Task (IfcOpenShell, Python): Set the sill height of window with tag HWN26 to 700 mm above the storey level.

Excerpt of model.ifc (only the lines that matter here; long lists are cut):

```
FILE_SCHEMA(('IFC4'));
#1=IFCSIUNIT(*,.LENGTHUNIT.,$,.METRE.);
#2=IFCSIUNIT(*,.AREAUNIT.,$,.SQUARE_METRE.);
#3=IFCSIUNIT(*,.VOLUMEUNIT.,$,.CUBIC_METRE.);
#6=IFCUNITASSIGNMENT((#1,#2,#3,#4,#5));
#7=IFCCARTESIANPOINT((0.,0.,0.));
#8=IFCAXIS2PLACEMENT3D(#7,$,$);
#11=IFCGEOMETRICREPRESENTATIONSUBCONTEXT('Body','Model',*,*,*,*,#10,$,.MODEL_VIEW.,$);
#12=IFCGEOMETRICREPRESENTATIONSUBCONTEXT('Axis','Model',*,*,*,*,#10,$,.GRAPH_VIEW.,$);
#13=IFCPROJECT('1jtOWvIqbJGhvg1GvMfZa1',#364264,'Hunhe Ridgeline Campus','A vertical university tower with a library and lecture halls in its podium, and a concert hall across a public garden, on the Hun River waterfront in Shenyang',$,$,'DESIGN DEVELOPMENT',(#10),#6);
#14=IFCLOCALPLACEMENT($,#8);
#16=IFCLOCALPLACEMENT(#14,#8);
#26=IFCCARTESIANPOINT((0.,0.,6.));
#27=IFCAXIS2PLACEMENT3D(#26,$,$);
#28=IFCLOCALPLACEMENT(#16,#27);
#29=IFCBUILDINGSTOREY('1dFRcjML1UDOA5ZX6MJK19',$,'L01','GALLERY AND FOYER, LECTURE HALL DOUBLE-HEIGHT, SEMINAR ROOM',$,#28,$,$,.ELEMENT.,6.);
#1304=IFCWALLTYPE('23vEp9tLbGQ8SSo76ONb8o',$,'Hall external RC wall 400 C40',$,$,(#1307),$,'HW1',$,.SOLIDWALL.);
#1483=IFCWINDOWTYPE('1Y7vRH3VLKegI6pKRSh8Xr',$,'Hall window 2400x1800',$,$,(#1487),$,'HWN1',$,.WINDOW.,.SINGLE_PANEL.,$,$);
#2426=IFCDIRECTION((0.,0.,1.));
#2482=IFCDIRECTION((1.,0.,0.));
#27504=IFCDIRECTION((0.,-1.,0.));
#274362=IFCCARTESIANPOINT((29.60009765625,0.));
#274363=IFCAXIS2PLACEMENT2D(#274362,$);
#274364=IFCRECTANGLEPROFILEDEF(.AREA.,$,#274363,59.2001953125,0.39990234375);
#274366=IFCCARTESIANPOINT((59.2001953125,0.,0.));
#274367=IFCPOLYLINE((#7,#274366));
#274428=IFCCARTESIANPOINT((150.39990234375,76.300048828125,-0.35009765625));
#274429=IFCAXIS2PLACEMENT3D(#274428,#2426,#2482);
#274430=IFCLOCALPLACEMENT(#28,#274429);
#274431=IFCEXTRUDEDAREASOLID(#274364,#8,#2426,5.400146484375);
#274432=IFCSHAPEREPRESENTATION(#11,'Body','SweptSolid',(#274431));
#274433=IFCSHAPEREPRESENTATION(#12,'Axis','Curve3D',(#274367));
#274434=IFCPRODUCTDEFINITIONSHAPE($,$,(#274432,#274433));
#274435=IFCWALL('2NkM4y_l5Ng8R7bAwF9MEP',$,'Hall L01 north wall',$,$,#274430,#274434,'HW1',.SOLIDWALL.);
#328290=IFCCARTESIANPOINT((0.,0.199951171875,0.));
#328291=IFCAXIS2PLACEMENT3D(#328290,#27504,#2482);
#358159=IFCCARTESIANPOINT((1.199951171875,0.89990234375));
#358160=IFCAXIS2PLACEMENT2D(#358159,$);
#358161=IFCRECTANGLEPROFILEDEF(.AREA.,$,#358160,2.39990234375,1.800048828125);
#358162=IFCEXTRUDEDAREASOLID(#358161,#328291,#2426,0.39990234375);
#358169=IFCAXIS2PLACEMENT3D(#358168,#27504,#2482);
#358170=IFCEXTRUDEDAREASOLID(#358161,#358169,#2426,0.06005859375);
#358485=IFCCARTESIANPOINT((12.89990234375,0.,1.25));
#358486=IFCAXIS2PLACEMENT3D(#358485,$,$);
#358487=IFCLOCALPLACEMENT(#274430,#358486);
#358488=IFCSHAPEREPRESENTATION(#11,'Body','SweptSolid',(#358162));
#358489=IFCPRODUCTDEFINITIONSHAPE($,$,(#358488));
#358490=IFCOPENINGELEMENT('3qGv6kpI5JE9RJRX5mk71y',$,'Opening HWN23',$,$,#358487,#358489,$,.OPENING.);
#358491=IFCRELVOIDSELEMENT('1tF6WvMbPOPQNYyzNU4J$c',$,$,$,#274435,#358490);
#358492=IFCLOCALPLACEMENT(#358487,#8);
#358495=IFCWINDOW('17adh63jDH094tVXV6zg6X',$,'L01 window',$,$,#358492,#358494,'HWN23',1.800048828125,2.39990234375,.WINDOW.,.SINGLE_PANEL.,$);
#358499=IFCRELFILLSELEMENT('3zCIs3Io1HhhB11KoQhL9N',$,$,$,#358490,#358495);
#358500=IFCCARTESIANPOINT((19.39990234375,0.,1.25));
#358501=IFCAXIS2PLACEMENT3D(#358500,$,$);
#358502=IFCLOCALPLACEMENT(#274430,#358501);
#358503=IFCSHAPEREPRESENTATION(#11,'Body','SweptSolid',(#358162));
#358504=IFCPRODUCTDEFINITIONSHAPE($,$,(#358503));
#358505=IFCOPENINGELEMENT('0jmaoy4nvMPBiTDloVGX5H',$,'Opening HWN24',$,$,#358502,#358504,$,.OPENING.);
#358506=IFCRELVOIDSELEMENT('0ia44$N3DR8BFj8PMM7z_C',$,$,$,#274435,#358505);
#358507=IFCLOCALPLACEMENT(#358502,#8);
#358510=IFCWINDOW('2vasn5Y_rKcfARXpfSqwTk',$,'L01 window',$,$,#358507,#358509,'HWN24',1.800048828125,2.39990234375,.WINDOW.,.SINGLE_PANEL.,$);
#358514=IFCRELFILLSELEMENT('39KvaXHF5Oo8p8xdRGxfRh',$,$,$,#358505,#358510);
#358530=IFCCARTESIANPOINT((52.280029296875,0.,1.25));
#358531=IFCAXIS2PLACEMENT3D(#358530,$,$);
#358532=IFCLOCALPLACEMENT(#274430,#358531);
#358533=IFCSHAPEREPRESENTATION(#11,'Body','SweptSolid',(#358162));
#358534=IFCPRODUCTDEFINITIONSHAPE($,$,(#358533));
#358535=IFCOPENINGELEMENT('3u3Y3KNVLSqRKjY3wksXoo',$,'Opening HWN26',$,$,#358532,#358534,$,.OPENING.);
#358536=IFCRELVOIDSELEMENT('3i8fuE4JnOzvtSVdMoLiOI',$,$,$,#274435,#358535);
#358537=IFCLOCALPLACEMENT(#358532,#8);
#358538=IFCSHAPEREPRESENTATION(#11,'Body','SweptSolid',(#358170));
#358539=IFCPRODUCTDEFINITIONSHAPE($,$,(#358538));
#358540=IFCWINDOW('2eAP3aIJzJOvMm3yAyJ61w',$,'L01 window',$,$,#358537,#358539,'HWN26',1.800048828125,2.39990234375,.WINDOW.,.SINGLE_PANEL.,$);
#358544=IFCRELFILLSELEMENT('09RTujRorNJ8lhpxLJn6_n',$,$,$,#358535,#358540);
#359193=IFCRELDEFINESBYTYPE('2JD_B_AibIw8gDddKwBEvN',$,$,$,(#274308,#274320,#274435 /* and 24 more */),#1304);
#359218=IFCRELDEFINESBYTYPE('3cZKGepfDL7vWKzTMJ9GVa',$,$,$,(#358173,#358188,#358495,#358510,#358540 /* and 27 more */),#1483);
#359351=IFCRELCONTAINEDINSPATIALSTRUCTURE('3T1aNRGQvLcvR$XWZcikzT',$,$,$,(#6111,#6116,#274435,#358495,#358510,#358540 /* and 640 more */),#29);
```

```python
import numpy as np
import ifcopenshell
import ifcopenshell.api.geometry
import ifcopenshell.geom
import ifcopenshell.util.element
import ifcopenshell.util.placement
import ifcopenshell.util.shape
import ifcopenshell.util.unit

model = ifcopenshell.open("model.ifc")
unit_scale = ifcopenshell.util.unit.calculate_unit_scale(model)

window = model.by_guid("2eAP3aIJzJOvMm3yAyJ61w")
opening = window.FillsVoids[0].RelatingOpeningElement
storey = ifcopenshell.util.element.get_container(window, ifc_class="IfcBuildingStorey")
level = ifcopenshell.util.placement.get_local_placement(storey.ObjectPlacement)[2, 3]

# The opening's origin need not be at the sill, so measure its lowest point.
shape = ifcopenshell.geom.create_shape(ifcopenshell.geom.settings(), opening)
bottom = ifcopenshell.util.shape.get_shape_bottom_elevation(shape, shape.geometry) / unit_scale
dz = level + 0.7 - bottom

shift = np.array([0.0, 0.0, dz])
# The window is placed relative to its opening, so it follows when the opening moves.
matrix = ifcopenshell.util.placement.get_local_placement(opening.ObjectPlacement)
matrix[:3, 3] += shift
ifcopenshell.api.geometry.edit_object_placement(
    model, product=opening, matrix=matrix, is_si=False, should_transform_children=True
)

print(f"moved by {dz * unit_scale:+.3f} m")

model.write("model-out.ifc")
```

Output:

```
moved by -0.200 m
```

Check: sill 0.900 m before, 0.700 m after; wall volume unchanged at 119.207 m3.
